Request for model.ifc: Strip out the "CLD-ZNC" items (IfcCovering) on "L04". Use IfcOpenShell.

First a look at what the model holds.

```python
import ifcopenshell
import ifcopenshell.util.element

model = ifcopenshell.open("model.ifc")
print(model.schema)
storey = next(s for s in model.by_type("IfcBuildingStorey") if s.Name == "L04")
coverings = [e for e in ifcopenshell.util.element.get_decomposition(storey) if e.is_a("IfcCovering")]
seen = {}
for e in coverings:
    element_type = ifcopenshell.util.element.get_type(e)
    name = element_type.Name if element_type not in (None, e) else None
    seen[name] = seen.get(name, 0) + 1
for name, count in sorted(seen.items(), key=str):
    print(count, "x", name)
```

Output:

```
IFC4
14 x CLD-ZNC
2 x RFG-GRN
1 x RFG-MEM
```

```python
import ifcopenshell
import ifcopenshell.api.root
import ifcopenshell.util.element

model = ifcopenshell.open("model.ifc")

storey = next(s for s in model.by_type("IfcBuildingStorey") if s.Name == "L04")
coverings = [e for e in ifcopenshell.util.element.get_decomposition(storey) if e.is_a("IfcCovering")]
targets = [e for e in coverings if (t := ifcopenshell.util.element.get_type(e)) not in (None, e) and t.Name == "CLD-ZNC"]

for e in targets:
    ifcopenshell.api.root.remove_product(model, product=e)
print(len(targets), "removed")

model.write("model-out.ifc")
```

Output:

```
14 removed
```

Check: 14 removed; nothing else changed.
